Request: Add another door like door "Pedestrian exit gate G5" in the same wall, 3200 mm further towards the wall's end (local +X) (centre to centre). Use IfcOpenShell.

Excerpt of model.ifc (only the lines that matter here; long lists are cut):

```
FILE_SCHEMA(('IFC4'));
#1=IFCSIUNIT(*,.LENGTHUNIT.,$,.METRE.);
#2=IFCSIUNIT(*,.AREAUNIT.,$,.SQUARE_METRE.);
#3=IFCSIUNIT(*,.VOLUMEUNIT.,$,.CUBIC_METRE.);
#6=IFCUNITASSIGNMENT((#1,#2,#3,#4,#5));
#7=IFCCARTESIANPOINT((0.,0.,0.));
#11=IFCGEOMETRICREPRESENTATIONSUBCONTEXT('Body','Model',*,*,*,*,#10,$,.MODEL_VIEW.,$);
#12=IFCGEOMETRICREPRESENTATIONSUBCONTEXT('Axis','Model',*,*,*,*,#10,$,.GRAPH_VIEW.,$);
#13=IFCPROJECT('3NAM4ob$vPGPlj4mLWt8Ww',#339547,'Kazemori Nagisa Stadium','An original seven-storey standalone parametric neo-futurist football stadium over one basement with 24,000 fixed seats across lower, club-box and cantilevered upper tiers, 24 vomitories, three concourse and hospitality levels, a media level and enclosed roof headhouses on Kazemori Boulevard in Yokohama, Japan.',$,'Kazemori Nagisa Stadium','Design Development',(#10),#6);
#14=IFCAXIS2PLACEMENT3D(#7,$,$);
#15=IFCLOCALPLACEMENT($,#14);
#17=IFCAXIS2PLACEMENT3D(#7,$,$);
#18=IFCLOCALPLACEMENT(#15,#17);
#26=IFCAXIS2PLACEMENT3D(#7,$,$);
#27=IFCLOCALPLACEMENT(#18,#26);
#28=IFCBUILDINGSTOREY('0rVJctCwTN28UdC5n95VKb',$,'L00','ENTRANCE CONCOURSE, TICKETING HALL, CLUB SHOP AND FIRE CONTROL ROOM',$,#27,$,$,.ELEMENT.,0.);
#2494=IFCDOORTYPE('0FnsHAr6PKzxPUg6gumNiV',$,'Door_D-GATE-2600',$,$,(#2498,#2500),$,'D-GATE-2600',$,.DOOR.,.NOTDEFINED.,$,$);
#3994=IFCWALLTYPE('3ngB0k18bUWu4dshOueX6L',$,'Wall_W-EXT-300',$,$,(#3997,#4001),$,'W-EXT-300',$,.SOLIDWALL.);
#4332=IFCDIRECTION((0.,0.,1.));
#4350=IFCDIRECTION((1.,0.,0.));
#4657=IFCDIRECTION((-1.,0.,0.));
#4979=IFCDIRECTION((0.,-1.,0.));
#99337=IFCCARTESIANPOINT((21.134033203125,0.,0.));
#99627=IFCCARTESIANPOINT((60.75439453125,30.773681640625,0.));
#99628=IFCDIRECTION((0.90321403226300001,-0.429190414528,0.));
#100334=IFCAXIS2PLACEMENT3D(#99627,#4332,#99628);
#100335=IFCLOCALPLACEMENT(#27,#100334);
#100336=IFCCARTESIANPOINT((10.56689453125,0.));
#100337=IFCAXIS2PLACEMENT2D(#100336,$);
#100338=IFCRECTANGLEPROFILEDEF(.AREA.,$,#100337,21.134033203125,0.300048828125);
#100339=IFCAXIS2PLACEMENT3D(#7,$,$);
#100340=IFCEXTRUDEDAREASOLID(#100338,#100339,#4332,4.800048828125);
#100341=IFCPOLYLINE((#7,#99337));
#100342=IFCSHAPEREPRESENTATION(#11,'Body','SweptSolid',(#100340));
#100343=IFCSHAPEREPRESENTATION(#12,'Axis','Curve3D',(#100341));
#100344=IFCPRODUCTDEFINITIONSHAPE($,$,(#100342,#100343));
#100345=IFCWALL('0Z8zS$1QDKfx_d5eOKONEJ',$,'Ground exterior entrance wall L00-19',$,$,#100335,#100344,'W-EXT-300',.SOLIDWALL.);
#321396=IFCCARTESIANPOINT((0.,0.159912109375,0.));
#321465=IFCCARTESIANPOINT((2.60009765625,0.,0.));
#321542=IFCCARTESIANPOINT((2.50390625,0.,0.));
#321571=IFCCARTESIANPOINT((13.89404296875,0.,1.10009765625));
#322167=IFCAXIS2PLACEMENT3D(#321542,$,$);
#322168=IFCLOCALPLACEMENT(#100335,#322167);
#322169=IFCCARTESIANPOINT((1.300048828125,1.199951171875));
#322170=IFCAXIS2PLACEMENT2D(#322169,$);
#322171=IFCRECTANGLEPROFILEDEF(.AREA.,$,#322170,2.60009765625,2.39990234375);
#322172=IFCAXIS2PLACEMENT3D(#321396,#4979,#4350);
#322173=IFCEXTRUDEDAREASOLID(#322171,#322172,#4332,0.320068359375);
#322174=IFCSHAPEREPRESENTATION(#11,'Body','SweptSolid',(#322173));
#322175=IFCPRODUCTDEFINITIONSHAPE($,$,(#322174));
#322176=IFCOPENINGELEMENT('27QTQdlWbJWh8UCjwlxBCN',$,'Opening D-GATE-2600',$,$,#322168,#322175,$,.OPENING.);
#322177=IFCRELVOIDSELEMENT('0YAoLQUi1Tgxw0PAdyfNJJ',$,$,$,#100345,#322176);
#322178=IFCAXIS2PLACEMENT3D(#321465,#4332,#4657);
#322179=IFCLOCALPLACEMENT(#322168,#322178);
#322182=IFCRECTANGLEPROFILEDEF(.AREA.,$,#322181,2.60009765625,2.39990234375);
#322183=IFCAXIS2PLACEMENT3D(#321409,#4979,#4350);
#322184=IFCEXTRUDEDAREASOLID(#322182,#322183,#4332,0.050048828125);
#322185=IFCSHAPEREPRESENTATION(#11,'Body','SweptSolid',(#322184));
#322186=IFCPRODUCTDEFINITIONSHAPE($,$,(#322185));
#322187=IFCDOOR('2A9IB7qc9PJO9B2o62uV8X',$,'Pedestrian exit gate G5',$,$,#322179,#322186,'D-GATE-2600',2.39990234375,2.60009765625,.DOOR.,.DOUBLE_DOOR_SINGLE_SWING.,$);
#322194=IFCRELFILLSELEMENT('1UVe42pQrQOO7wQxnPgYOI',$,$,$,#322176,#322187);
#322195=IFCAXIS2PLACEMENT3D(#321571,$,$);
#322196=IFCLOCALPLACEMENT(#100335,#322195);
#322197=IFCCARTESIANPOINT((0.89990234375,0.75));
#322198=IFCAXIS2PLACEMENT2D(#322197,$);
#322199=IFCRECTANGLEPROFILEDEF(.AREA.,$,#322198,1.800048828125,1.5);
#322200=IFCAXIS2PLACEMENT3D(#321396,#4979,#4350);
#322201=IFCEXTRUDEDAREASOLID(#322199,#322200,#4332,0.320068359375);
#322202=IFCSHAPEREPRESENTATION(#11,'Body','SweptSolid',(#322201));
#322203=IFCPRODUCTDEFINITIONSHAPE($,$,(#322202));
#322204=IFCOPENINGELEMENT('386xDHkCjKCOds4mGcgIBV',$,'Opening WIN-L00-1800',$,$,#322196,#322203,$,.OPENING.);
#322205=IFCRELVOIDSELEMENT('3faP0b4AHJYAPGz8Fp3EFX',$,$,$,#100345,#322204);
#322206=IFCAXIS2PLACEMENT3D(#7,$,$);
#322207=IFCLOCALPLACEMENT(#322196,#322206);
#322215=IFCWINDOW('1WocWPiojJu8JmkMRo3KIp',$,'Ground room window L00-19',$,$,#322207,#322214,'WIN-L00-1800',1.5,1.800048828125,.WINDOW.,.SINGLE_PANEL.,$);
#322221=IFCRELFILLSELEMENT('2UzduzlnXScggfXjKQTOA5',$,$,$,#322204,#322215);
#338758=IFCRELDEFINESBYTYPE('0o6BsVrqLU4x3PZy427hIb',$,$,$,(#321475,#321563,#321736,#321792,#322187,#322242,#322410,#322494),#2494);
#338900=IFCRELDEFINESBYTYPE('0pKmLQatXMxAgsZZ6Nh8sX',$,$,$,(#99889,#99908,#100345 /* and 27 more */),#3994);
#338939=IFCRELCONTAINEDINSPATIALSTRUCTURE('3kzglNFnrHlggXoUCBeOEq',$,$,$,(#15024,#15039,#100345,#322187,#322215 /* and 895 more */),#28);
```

```python
import ifcopenshell
import ifcopenshell.api.feature
import ifcopenshell.api.geometry
import ifcopenshell.api.root
import ifcopenshell.geom
import ifcopenshell.util.element
import ifcopenshell.util.placement
import ifcopenshell.util.shape
import ifcopenshell.util.unit

model = ifcopenshell.open("model.ifc")
unit_scale = ifcopenshell.util.unit.calculate_unit_scale(model)
settings = ifcopenshell.geom.settings()


def volume(element):
    """Net volume in cubic metres, openings subtracted."""
    shape = ifcopenshell.geom.create_shape(settings, element)
    return ifcopenshell.util.shape.get_volume(shape.geometry)


door = model.by_id(322187)
opening = door.FillsVoids[0].RelatingOpeningElement
wall = opening.VoidsElements[0].RelatingBuildingElement
before = volume(wall)
shift = ifcopenshell.util.placement.get_local_placement(wall.ObjectPlacement)[:3, 0] * 3.2 / unit_scale

# copy_class copies the void relationship, type, container and properties, but no geometry.
new_opening = ifcopenshell.api.root.copy_class(model, product=opening)
new_opening.Representation = ifcopenshell.util.element.copy_deep(
    model, opening.Representation, exclude=["IfcGeometricRepresentationContext", "IfcRepresentationMap"]
)
new_door = ifcopenshell.api.root.copy_class(model, product=door)
new_door.Representation = ifcopenshell.util.element.copy_deep(
    model, door.Representation, exclude=["IfcGeometricRepresentationContext", "IfcRepresentationMap"]
)
new_door.Tag = None
ifcopenshell.api.feature.add_filling(model, opening=new_opening, element=new_door)

for old, new in ((opening, new_opening), (door, new_door)):
    matrix = ifcopenshell.util.placement.get_local_placement(old.ObjectPlacement)
    matrix[:3, 3] += shift
    ifcopenshell.api.geometry.edit_object_placement(model, product=new, matrix=matrix, is_si=False)

after = volume(wall)

print(f"wall volume {before:.3f} -> {after:.3f} m3")

model.write("model_edited.ifc")
```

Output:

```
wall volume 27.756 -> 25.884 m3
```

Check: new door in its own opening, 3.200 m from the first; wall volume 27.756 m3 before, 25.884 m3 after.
